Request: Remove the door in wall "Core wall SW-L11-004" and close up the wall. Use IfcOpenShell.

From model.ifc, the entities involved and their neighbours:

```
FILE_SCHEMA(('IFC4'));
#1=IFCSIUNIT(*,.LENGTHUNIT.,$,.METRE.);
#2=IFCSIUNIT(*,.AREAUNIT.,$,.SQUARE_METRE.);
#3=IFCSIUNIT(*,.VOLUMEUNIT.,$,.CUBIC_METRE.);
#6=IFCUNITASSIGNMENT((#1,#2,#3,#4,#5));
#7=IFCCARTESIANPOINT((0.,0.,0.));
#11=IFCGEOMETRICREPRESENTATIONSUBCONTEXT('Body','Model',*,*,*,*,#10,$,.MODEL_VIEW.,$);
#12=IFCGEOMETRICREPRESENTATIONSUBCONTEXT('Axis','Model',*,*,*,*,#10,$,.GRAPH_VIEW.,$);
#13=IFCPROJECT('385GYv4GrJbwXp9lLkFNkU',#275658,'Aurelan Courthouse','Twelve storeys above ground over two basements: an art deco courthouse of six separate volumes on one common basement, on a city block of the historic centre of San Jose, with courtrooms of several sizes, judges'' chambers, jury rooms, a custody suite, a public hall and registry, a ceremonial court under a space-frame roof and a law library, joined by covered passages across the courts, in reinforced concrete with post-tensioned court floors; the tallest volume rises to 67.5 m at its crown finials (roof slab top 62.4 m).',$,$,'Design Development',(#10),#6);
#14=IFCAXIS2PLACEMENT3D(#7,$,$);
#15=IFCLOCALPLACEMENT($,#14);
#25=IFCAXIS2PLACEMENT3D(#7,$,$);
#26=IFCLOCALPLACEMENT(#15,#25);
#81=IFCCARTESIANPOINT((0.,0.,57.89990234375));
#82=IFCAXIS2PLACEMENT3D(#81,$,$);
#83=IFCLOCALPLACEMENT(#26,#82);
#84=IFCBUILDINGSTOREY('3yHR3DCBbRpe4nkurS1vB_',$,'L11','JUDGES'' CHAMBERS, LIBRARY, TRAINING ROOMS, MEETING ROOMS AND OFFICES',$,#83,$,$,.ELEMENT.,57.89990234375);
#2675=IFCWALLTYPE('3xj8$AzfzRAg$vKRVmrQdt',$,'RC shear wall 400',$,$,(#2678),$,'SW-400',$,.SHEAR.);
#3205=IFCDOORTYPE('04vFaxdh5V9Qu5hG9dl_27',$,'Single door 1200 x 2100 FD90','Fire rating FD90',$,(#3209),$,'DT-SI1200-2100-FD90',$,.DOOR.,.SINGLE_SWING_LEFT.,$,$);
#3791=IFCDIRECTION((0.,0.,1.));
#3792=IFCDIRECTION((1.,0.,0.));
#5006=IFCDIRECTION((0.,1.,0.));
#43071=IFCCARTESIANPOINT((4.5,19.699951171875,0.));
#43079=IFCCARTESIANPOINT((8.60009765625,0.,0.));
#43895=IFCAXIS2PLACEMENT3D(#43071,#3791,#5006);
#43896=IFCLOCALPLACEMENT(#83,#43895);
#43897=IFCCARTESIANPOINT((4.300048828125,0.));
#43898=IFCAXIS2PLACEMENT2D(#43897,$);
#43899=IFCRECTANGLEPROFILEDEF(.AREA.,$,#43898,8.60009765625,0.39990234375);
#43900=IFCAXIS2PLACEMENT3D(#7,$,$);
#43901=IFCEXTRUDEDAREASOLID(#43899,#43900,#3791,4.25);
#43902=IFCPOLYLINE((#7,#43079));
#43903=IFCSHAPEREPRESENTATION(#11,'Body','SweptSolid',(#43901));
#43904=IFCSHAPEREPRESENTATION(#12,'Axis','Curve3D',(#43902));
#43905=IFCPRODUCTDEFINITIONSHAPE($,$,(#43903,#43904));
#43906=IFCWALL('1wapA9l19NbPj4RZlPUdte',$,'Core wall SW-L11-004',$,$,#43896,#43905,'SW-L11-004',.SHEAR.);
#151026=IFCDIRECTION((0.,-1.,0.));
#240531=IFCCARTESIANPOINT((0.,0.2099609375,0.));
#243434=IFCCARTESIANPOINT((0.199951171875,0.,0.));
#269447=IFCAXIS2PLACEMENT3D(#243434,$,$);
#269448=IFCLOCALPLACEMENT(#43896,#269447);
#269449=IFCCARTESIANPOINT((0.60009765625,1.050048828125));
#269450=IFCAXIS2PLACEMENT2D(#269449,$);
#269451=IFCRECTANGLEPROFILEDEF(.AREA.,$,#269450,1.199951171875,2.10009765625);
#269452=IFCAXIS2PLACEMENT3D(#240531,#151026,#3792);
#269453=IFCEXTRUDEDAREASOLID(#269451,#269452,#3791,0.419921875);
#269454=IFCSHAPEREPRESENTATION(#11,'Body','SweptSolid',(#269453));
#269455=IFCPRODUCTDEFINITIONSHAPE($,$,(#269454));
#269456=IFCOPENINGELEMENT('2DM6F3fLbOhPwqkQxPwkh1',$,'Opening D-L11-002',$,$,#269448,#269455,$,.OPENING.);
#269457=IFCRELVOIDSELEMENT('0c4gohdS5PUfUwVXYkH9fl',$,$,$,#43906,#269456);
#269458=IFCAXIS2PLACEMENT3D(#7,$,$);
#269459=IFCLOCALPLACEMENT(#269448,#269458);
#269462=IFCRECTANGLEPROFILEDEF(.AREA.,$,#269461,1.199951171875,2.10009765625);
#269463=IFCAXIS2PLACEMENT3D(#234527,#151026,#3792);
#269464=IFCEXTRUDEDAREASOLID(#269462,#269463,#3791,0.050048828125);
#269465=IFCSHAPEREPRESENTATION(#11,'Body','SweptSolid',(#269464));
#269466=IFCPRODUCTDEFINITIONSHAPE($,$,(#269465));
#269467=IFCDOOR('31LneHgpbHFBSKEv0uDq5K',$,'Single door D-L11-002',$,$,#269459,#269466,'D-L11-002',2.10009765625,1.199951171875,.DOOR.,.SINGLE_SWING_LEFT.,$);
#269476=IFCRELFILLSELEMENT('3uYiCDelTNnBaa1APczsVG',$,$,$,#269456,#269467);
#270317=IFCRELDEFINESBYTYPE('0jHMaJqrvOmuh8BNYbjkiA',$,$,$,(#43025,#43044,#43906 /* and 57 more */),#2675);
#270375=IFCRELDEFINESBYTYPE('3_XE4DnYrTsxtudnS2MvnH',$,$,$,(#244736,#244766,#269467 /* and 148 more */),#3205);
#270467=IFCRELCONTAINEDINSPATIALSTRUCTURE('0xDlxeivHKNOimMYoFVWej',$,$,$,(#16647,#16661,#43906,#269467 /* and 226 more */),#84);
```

```python
import ifcopenshell
import ifcopenshell.api.feature
import ifcopenshell.api.root
import ifcopenshell.geom
import ifcopenshell.util.shape

model = ifcopenshell.open("model.ifc")
settings = ifcopenshell.geom.settings()


def volume(element):
    """Net volume in cubic metres, openings subtracted."""
    shape = ifcopenshell.geom.create_shape(settings, element)
    return ifcopenshell.util.shape.get_volume(shape.geometry)


door = model.by_guid("31LneHgpbHFBSKEv0uDq5K")
opening = door.FillsVoids[0].RelatingOpeningElement
wall = opening.VoidsElements[0].RelatingBuildingElement
before = volume(wall)

ifcopenshell.api.root.remove_product(model, product=door)
ifcopenshell.api.feature.remove_feature(model, feature=opening)

after = volume(wall)

print(f"wall volume {before:.3f} -> {after:.3f} m3")

model.write("model-out.ifc")
```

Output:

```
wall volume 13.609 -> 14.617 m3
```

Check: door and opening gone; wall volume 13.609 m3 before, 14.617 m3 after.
